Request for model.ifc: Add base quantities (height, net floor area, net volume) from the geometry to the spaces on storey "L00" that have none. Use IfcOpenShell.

First a look at what the model holds.

```python
import ifcopenshell
import ifcopenshell.util.element
import ifcopenshell.util.unit

model = ifcopenshell.open("model.ifc")
print(model.schema)
for unit_type in ("LENGTHUNIT", "AREAUNIT", "VOLUMEUNIT"):
    print(unit_type, ifcopenshell.util.unit.calculate_unit_scale(model, unit_type))
storey = next(s for s in model.by_type("IfcBuildingStorey") if s.Name == "L00")
spaces = [e for e in ifcopenshell.util.element.get_decomposition(storey) if e.is_a("IfcSpace")]
for e in sorted(spaces, key=lambda e: e.id()):
    print(e.id(), e.is_a(), e.Name, list(ifcopenshell.util.element.get_psets(e, qtos_only=True)), sep=" | ")
```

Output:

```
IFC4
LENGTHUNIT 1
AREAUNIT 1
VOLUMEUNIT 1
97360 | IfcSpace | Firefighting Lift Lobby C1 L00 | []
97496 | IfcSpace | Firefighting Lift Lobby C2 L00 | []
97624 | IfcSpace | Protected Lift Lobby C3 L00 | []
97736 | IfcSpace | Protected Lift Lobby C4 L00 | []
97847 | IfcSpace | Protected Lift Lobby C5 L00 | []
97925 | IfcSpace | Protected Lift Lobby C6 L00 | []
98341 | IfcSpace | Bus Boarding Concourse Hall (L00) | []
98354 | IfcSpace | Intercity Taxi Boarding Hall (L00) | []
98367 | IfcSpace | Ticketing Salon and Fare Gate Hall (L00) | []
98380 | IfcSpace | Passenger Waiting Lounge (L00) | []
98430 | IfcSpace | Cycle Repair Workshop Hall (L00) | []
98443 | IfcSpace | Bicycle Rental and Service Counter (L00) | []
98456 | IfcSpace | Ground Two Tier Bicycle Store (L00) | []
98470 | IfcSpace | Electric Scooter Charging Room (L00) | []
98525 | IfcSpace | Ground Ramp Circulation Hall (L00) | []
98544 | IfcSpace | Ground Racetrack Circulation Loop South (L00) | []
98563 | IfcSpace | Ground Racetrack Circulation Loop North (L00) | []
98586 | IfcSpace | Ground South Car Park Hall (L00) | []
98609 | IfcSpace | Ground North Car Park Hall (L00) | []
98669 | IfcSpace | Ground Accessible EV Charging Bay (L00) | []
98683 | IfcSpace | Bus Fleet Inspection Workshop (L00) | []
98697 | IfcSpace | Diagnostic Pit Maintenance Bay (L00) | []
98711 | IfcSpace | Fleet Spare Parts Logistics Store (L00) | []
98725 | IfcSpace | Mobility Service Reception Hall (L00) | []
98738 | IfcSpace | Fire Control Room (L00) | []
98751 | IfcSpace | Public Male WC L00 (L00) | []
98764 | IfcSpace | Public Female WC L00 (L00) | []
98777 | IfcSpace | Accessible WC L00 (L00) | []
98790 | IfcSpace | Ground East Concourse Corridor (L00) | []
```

```python
import ifcopenshell
import ifcopenshell.api.pset
import ifcopenshell.geom
import ifcopenshell.util.element
import ifcopenshell.util.shape
import ifcopenshell.util.unit

model = ifcopenshell.open("model.ifc")
unit_scale = ifcopenshell.util.unit.calculate_unit_scale(model)
area_scale = ifcopenshell.util.unit.calculate_unit_scale(model, "AREAUNIT")
volume_scale = ifcopenshell.util.unit.calculate_unit_scale(model, "VOLUMEUNIT")
settings = ifcopenshell.geom.settings()

storey = next(s for s in model.by_type("IfcBuildingStorey") if s.Name == "L00")
spaces = [e for e in ifcopenshell.util.element.get_decomposition(storey) if e.is_a("IfcSpace")]

for e in sorted(spaces, key=lambda e: e.id()):
    if ifcopenshell.util.element.get_psets(e, qtos_only=True, should_inherit=False):
        continue
    # Geometry comes back in metres, in the element's own axes.
    shape = ifcopenshell.geom.create_shape(settings, e)
    values = {
        "Height": ifcopenshell.util.shape.get_z(shape.geometry) / unit_scale,
        "NetFloorArea": ifcopenshell.util.shape.get_footprint_area(shape.geometry) / area_scale,
        "NetVolume": ifcopenshell.util.shape.get_volume(shape.geometry) / volume_scale,
    }
    qto = ifcopenshell.api.pset.add_qto(model, product=e, name="Qto_SpaceBaseQuantities")
    ifcopenshell.api.pset.edit_qto(model, qto=qto, properties=values)
    print(e.id(), {k: round(v, 3) for k, v in values.items()})

model.write("model_rev.ifc")
```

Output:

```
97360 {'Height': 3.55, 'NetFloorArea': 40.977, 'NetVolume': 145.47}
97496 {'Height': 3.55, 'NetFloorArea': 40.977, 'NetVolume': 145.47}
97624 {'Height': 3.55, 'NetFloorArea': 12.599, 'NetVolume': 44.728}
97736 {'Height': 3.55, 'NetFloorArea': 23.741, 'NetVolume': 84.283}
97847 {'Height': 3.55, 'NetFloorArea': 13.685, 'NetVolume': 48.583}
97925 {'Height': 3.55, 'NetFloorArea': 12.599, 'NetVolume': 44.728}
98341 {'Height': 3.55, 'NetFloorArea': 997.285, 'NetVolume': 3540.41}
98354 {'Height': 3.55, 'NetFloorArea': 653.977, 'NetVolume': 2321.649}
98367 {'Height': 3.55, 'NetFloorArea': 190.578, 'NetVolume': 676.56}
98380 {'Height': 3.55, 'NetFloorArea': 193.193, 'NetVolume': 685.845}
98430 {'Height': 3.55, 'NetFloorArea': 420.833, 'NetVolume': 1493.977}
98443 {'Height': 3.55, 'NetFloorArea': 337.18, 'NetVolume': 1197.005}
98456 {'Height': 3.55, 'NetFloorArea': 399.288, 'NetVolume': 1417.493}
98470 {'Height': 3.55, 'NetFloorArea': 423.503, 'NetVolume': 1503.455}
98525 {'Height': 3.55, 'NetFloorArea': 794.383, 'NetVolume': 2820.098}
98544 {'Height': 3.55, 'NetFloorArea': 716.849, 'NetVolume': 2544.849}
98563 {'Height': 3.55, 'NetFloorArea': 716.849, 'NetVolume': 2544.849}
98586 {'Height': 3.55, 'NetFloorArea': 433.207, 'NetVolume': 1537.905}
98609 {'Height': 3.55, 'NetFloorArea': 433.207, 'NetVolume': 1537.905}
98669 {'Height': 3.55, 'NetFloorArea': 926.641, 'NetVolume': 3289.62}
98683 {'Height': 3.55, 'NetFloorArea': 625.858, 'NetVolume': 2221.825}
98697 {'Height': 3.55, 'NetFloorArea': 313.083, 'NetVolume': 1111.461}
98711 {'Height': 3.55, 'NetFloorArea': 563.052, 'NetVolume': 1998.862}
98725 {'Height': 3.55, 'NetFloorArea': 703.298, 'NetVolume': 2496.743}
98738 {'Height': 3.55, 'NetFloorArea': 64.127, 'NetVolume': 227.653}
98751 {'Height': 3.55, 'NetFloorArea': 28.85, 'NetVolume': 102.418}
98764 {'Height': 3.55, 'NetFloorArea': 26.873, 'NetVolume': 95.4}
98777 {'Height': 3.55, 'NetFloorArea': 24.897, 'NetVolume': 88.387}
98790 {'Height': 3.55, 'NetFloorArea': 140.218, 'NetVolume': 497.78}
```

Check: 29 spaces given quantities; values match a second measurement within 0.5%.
